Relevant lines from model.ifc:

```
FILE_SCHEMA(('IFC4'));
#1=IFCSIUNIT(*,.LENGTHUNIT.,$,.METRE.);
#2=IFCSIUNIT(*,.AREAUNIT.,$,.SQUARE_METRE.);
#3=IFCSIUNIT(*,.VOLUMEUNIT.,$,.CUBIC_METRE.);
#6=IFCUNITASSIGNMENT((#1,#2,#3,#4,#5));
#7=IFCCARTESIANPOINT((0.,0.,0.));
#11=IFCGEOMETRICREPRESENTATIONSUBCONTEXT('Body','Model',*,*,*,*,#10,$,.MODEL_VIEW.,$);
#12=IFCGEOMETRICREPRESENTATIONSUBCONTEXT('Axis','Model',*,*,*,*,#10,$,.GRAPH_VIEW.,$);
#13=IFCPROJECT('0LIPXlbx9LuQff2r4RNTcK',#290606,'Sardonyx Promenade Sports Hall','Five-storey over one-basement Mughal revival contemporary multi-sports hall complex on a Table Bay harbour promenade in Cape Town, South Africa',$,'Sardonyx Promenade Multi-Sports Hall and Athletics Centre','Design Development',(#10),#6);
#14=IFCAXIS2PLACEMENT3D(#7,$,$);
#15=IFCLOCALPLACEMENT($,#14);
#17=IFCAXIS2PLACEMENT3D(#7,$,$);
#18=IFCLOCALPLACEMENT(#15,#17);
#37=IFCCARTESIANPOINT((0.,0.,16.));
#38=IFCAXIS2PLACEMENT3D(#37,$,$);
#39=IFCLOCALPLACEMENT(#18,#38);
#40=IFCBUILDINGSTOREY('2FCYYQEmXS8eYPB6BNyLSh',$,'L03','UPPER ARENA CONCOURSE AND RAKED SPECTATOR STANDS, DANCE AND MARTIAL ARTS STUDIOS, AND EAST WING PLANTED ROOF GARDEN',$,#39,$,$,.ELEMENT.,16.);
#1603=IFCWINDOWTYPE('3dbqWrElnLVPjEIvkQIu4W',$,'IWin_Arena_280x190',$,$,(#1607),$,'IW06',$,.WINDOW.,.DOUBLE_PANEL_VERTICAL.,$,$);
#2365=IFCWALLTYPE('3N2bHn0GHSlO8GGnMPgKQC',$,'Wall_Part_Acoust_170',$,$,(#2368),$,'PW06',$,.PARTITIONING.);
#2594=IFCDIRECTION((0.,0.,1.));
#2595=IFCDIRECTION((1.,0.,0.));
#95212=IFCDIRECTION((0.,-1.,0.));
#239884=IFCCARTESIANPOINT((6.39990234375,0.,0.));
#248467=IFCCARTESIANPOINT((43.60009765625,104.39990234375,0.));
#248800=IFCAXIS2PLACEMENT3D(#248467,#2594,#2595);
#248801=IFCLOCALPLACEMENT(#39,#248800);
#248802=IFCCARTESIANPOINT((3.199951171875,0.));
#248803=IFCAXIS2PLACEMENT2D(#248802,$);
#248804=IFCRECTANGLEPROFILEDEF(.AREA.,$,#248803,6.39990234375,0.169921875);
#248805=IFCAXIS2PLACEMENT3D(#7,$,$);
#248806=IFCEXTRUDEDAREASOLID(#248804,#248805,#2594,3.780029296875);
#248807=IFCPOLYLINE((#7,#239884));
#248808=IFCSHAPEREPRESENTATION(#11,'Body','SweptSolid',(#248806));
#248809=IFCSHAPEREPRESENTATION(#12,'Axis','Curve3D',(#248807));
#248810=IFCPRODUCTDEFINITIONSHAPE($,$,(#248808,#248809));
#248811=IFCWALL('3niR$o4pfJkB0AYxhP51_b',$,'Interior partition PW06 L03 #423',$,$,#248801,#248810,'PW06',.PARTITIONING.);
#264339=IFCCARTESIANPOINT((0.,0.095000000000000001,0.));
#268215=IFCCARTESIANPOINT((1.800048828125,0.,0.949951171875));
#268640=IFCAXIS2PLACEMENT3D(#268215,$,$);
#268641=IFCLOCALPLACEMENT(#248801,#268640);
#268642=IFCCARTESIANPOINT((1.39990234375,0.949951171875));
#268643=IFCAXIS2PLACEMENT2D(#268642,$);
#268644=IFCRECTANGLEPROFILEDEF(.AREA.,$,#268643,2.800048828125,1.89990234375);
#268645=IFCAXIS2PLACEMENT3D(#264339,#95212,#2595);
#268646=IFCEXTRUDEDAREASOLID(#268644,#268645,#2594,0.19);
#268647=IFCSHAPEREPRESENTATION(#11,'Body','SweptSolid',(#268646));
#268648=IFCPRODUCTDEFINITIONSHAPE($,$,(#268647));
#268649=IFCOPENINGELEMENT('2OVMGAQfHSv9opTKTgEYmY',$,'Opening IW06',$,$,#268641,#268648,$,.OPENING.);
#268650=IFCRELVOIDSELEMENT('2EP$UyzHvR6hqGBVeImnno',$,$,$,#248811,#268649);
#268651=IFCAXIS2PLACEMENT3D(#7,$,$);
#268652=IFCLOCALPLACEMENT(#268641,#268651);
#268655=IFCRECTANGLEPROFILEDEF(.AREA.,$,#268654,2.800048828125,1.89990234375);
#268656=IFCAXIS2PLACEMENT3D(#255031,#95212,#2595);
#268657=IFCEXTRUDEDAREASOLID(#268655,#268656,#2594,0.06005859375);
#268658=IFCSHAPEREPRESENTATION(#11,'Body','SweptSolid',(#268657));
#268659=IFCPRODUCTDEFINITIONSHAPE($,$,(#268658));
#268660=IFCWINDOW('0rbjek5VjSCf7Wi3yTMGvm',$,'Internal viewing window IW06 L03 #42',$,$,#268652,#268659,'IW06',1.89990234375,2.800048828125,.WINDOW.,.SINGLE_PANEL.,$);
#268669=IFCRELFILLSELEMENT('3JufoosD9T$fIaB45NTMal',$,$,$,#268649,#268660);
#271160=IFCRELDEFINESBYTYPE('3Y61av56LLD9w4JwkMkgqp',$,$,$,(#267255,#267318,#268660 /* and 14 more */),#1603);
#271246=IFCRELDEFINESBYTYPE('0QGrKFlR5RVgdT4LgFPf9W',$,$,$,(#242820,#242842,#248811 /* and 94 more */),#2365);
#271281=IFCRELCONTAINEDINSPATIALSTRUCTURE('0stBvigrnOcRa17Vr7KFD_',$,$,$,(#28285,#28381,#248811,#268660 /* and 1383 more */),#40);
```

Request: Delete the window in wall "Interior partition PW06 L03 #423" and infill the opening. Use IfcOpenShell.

```python
import ifcopenshell
import ifcopenshell.api.feature
import ifcopenshell.api.root
import ifcopenshell.geom
import ifcopenshell.util.shape

model = ifcopenshell.open("model.ifc")
settings = ifcopenshell.geom.settings()


def volume(element):
    """Net volume in cubic metres, openings subtracted."""
    shape = ifcopenshell.geom.create_shape(settings, element)
    return ifcopenshell.util.shape.get_volume(shape.geometry)


window = model.by_guid("0rbjek5VjSCf7Wi3yTMGvm")
opening = window.FillsVoids[0].RelatingOpeningElement
wall = opening.VoidsElements[0].RelatingBuildingElement
before = volume(wall)

ifcopenshell.api.root.remove_product(model, product=window)
ifcopenshell.api.feature.remove_feature(model, feature=opening)

after = volume(wall)

print(f"wall volume {before:.3f} -> {after:.3f} m3")

model.write("model_edited.ifc")
```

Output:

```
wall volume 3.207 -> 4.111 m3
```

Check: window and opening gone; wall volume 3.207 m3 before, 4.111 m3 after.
